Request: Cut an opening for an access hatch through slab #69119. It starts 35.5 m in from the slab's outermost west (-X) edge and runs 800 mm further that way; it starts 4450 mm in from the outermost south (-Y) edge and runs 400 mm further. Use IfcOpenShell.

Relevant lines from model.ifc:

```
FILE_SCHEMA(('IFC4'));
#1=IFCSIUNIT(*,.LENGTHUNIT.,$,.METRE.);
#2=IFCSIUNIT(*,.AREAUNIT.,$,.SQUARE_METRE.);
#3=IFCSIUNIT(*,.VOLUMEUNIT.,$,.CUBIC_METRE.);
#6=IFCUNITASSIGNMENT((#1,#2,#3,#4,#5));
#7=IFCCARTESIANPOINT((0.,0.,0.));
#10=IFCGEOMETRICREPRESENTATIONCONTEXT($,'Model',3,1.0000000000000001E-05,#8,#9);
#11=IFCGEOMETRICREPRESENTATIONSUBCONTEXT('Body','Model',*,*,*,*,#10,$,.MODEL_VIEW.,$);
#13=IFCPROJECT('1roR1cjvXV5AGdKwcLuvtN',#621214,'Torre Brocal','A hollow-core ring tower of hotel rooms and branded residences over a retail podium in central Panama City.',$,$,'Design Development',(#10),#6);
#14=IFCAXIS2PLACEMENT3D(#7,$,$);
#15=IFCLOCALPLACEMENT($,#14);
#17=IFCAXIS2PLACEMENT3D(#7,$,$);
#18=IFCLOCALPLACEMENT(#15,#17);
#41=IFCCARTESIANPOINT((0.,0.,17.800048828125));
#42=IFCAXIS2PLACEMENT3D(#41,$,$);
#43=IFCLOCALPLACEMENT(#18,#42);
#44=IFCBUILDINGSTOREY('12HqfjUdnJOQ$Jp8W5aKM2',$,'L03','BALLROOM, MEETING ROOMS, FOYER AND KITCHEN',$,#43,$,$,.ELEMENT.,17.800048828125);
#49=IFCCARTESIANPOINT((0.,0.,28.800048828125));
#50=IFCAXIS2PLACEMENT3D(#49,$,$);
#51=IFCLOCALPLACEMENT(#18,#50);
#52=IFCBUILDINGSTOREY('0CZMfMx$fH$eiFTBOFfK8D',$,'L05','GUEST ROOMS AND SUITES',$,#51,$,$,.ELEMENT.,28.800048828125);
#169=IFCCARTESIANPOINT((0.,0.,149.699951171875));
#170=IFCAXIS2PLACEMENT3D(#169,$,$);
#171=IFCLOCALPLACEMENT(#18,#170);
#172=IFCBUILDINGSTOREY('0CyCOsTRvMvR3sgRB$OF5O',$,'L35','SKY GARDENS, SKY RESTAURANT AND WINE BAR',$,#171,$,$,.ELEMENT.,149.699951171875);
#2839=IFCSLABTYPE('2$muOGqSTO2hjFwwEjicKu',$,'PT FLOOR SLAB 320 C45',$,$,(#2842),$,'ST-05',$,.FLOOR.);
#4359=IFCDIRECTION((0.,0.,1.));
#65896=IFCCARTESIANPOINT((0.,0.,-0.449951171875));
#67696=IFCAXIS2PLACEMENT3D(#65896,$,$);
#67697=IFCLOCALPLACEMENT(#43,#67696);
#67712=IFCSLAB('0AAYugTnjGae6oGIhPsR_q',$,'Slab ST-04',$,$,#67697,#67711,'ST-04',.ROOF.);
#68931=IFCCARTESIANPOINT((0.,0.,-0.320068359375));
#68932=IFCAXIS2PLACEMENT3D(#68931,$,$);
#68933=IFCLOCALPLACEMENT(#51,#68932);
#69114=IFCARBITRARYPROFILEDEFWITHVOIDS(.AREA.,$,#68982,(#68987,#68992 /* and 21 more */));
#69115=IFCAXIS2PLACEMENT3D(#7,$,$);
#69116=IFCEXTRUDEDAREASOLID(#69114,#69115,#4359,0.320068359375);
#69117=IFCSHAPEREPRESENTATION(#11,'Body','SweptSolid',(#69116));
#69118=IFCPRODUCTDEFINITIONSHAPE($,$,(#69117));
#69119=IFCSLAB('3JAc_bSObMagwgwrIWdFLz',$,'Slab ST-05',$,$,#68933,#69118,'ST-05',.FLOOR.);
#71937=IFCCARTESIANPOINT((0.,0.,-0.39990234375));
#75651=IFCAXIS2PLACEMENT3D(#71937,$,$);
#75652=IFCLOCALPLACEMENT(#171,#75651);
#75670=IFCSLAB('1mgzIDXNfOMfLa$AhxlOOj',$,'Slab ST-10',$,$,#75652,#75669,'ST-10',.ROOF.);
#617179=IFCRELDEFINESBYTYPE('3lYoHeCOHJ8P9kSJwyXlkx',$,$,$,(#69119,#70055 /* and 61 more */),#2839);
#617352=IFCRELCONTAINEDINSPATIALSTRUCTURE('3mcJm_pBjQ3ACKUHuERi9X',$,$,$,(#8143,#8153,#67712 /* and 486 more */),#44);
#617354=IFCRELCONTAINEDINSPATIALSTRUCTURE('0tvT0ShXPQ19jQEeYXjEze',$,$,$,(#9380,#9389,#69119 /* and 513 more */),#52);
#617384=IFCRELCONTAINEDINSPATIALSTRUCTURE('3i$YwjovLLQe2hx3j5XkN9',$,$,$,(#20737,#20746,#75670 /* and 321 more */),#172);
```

```python
import numpy as np
import ifcopenshell
import ifcopenshell.api.feature
import ifcopenshell.api.geometry
import ifcopenshell.api.root
import ifcopenshell.geom
import ifcopenshell.util.placement
import ifcopenshell.util.representation
import ifcopenshell.util.shape
import ifcopenshell.util.unit

model = ifcopenshell.open("model.ifc")
unit_scale = ifcopenshell.util.unit.calculate_unit_scale(model)
settings = ifcopenshell.geom.settings()


def volume(element):
    """Net volume in cubic metres, openings subtracted."""
    shape = ifcopenshell.geom.create_shape(settings, element)
    return ifcopenshell.util.shape.get_volume(shape.geometry)


slab = model.by_guid("3JAc_bSObMagwgwrIWdFLz")
before = volume(slab)

# Extent in the slab's own axes, in metres. The edges named are its -X and -Y sides.
slab_shape = ifcopenshell.geom.create_shape(settings, slab)
vertices = ifcopenshell.util.shape.get_vertices(slab_shape.geometry)
x_min, y_min, bottom = vertices.min(axis=0)
top = vertices[:, 2].max()

opening = ifcopenshell.api.root.create_entity(model, ifc_class="IfcOpeningElement", name="Access hatch opening", predefined_type="OPENING")
context = ifcopenshell.util.representation.get_context(model, "Model", "Body", "MODEL_VIEW")
width, depth = 0.8, 0.4
outline = [(0.0, 0.0), (width, 0.0), (width, depth), (0.0, depth), (0.0, 0.0)]
# Overshoot both faces by 50 mm so the cut is clean.
shape = ifcopenshell.api.geometry.add_slab_representation(
    model, context=context, depth=top - bottom + 0.1, polyline=outline
)
ifcopenshell.api.geometry.assign_representation(model, product=opening, representation=shape)

matrix = ifcopenshell.util.placement.get_local_placement(slab.ObjectPlacement)
matrix[:, 3] = matrix @ np.append(np.array([x_min + 35.5, y_min + 4.45, bottom - 0.05]) / unit_scale, 1.0)
ifcopenshell.api.geometry.edit_object_placement(model, product=opening, matrix=matrix, is_si=False)
ifcopenshell.api.feature.add_feature(model, feature=opening, element=slab)

after = volume(slab)

print(f"slab volume {before:.3f} -> {after:.3f} m3")

model.write("model_v2.ifc")
```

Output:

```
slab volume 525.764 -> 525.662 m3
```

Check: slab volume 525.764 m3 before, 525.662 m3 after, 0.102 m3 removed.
